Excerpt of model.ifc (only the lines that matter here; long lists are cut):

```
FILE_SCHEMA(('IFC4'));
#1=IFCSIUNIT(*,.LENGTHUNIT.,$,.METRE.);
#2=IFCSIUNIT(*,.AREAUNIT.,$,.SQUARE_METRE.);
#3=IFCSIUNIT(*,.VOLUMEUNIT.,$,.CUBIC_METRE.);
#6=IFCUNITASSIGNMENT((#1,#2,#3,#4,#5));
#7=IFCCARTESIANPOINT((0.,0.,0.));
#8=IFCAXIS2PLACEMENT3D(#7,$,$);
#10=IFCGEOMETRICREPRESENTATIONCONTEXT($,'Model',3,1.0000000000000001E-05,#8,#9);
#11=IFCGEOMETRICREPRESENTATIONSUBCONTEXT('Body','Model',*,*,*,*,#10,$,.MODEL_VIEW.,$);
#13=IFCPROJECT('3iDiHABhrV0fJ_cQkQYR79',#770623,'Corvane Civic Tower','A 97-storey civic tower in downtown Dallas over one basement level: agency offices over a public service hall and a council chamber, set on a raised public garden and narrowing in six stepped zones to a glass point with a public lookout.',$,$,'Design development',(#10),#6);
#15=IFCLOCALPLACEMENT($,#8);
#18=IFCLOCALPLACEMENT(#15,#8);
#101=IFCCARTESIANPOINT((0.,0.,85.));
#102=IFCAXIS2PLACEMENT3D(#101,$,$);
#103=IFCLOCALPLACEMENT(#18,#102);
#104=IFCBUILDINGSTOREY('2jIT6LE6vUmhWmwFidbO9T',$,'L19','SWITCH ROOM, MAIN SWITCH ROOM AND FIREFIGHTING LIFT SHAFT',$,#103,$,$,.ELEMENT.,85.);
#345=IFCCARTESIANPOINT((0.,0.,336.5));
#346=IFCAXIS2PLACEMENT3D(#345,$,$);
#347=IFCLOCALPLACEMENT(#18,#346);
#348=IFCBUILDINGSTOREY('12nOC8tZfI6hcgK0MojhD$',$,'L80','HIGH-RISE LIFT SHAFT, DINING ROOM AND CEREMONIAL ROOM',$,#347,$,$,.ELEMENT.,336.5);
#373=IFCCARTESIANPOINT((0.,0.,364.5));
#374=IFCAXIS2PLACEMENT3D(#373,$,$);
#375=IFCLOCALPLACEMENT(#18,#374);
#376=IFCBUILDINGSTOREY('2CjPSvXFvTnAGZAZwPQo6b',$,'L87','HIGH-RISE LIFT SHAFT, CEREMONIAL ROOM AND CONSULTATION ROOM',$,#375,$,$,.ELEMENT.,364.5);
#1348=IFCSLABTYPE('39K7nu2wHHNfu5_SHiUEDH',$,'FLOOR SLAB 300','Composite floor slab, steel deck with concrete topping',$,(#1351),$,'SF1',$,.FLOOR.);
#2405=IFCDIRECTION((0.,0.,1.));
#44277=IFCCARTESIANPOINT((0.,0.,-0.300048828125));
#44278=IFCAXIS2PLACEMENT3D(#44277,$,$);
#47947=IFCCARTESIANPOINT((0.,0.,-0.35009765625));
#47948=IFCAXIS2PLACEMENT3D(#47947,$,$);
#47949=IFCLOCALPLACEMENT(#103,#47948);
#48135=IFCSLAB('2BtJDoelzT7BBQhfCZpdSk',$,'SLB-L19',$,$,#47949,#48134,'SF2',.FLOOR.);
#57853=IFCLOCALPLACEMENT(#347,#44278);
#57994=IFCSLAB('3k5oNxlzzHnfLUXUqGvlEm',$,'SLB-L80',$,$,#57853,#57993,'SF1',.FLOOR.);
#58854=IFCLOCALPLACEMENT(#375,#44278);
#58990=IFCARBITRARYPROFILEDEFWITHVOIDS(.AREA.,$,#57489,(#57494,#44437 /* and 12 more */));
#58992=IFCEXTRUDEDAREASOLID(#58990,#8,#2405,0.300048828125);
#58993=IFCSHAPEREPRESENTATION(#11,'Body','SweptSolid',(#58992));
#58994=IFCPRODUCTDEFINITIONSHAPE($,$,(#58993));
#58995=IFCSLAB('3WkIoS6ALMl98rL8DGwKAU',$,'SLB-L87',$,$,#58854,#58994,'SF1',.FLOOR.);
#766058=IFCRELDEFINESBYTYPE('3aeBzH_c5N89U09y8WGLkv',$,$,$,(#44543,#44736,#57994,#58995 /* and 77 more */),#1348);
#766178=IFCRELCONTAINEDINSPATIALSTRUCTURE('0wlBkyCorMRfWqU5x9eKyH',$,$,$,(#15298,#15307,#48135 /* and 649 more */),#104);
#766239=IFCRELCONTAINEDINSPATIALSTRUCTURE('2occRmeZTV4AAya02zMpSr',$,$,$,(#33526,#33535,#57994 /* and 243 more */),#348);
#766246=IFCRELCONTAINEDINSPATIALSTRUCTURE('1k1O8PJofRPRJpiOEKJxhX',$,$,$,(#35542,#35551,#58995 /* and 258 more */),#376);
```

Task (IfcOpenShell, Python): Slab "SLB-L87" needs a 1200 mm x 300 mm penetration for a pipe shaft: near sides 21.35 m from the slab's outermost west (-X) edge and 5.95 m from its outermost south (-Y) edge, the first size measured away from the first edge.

```python
import numpy as np
import ifcopenshell
import ifcopenshell.api.feature
import ifcopenshell.api.geometry
import ifcopenshell.api.root
import ifcopenshell.geom
import ifcopenshell.util.placement
import ifcopenshell.util.representation
import ifcopenshell.util.shape
import ifcopenshell.util.unit

model = ifcopenshell.open("model.ifc")
unit_scale = ifcopenshell.util.unit.calculate_unit_scale(model)
settings = ifcopenshell.geom.settings()


def volume(element):
    """Net volume in cubic metres, openings subtracted."""
    shape = ifcopenshell.geom.create_shape(settings, element)
    return ifcopenshell.util.shape.get_volume(shape.geometry)


slab = model.by_id(58995)
before = volume(slab)

# Extent in the slab's own axes, in metres. The edges named are its -X and -Y sides.
slab_shape = ifcopenshell.geom.create_shape(settings, slab)
vertices = ifcopenshell.util.shape.get_vertices(slab_shape.geometry)
x_min, y_min, bottom = vertices.min(axis=0)
top = vertices[:, 2].max()

opening = ifcopenshell.api.root.create_entity(model, ifc_class="IfcOpeningElement", name="Pipe shaft opening", predefined_type="OPENING")
context = ifcopenshell.util.representation.get_context(model, "Model", "Body", "MODEL_VIEW")
width, depth = 1.2, 0.3
outline = [(0.0, 0.0), (width, 0.0), (width, depth), (0.0, depth), (0.0, 0.0)]
# Overshoot both faces by 50 mm so the cut is clean.
shape = ifcopenshell.api.geometry.add_slab_representation(
    model, context=context, depth=top - bottom + 0.1, polyline=outline
)
ifcopenshell.api.geometry.assign_representation(model, product=opening, representation=shape)

matrix = ifcopenshell.util.placement.get_local_placement(slab.ObjectPlacement)
matrix[:, 3] = matrix @ np.append(np.array([x_min + 21.35, y_min + 5.95, bottom - 0.05]) / unit_scale, 1.0)
ifcopenshell.api.geometry.edit_object_placement(model, product=opening, matrix=matrix, is_si=False)
ifcopenshell.api.feature.add_feature(model, feature=opening, element=slab)

after = volume(slab)

print(f"slab volume {before:.3f} -> {after:.3f} m3")

model.write("model_edited.ifc")
```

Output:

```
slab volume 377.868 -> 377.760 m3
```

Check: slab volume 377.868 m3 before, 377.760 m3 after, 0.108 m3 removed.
